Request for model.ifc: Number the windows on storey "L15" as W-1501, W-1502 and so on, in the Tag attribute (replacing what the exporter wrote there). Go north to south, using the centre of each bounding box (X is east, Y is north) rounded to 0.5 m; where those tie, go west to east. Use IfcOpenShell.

First a look at what the model holds.

```python
import ifcopenshell
import ifcopenshell.util.element
import ifcopenshell.util.placement

model = ifcopenshell.open("model.ifc")
print(model.schema)
storey = next(s for s in model.by_type("IfcBuildingStorey") if s.Name == "L15")
windows = [e for e in ifcopenshell.util.element.get_decomposition(storey) if e.is_a("IfcWindow")]
for e in sorted(windows, key=lambda e: e.id()):
    origin = ifcopenshell.util.placement.get_local_placement(e.ObjectPlacement)[:3, 3]
    print(e.id(), e.Tag, e.Name, origin.round(2) + 0.0, sep=" | ")
```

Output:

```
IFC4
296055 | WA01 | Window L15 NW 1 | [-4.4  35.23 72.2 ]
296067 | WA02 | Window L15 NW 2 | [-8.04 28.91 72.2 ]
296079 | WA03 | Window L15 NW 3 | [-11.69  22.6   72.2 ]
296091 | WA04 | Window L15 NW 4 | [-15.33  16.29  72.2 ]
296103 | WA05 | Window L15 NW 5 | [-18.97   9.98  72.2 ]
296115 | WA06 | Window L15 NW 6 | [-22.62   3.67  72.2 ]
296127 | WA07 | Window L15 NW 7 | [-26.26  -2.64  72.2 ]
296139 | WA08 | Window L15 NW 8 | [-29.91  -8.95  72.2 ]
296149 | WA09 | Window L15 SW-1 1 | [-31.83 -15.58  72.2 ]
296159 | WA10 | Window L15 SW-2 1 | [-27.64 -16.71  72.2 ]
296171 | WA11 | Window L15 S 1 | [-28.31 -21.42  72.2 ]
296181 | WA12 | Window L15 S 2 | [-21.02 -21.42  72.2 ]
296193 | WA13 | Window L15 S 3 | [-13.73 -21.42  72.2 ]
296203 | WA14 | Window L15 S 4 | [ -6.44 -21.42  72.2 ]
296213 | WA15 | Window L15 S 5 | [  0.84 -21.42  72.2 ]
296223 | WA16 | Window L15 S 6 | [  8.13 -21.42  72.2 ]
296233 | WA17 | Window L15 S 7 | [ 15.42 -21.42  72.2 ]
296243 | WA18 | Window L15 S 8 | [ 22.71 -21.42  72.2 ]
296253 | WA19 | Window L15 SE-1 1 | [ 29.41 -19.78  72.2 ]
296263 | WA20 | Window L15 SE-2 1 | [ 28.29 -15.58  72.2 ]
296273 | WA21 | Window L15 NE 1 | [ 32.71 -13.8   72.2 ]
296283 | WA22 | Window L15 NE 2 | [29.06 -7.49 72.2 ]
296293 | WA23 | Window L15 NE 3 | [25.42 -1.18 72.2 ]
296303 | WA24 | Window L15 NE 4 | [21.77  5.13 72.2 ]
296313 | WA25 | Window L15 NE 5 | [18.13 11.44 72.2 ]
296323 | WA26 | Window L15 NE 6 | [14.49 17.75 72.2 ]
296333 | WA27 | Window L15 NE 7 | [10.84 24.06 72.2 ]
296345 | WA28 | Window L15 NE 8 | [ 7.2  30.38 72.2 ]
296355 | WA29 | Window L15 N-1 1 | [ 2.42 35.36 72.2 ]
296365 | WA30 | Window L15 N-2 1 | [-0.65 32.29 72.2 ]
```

```python
import ifcopenshell
import ifcopenshell.geom
import ifcopenshell.util.element
import ifcopenshell.util.shape

model = ifcopenshell.open("model.ifc")
settings = ifcopenshell.geom.settings()
settings.set("use-world-coords", True)


def centre(element):
    shape = ifcopenshell.geom.create_shape(settings, element)
    return ifcopenshell.util.shape.get_bbox_centroid(shape.geometry)


storey = next(s for s in model.by_type("IfcBuildingStorey") if s.Name == "L15")
windows = [e for e in ifcopenshell.util.element.get_decomposition(storey) if e.is_a("IfcWindow")]

# Insertion points can sit at a corner or the storey origin, so sort by the geometry (in metres).
centres = {e: centre(e) for e in windows}
windows.sort(key=lambda e: (-round(centres[e][1] / 0.5), centres[e][0]))

for i, e in enumerate(windows, start=1):
    number = f"W-15{i:02d}"
    e.Tag = number
    print(e.id(), number)

model.write("model_updated.ifc")
```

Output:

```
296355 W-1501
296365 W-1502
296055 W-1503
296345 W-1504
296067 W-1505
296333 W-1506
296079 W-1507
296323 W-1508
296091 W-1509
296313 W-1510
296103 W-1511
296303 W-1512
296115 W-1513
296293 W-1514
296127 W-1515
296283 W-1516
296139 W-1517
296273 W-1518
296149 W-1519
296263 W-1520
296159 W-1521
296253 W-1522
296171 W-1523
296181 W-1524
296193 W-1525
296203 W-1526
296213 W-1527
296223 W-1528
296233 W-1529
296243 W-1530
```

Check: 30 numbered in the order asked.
